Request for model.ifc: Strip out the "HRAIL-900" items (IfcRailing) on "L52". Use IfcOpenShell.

First a look at what the model holds.

```python
import ifcopenshell
import ifcopenshell.util.element

model = ifcopenshell.open("model.ifc")
print(model.schema)
storey = next(s for s in model.by_type("IfcBuildingStorey") if s.Name == "L52")
railings = [e for e in ifcopenshell.util.element.get_decomposition(storey) if e.is_a("IfcRailing")]
seen = {}
for e in railings:
    element_type = ifcopenshell.util.element.get_type(e)
    name = element_type.Name if element_type not in (None, e) else None
    seen[name] = seen.get(name, 0) + 1
for name, count in sorted(seen.items(), key=str):
    print(count, "x", name)
```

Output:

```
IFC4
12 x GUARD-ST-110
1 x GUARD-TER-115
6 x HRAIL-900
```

```python
import ifcopenshell
import ifcopenshell.api.root
import ifcopenshell.util.element

model = ifcopenshell.open("model.ifc")

storey = next(s for s in model.by_type("IfcBuildingStorey") if s.Name == "L52")
railings = [e for e in ifcopenshell.util.element.get_decomposition(storey) if e.is_a("IfcRailing")]
targets = [e for e in railings if (t := ifcopenshell.util.element.get_type(e)) not in (None, e) and t.Name == "HRAIL-900"]

for e in targets:
    ifcopenshell.api.root.remove_product(model, product=e)
print(len(targets), "removed")

model.write("model_v2.ifc")
```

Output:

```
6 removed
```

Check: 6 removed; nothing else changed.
